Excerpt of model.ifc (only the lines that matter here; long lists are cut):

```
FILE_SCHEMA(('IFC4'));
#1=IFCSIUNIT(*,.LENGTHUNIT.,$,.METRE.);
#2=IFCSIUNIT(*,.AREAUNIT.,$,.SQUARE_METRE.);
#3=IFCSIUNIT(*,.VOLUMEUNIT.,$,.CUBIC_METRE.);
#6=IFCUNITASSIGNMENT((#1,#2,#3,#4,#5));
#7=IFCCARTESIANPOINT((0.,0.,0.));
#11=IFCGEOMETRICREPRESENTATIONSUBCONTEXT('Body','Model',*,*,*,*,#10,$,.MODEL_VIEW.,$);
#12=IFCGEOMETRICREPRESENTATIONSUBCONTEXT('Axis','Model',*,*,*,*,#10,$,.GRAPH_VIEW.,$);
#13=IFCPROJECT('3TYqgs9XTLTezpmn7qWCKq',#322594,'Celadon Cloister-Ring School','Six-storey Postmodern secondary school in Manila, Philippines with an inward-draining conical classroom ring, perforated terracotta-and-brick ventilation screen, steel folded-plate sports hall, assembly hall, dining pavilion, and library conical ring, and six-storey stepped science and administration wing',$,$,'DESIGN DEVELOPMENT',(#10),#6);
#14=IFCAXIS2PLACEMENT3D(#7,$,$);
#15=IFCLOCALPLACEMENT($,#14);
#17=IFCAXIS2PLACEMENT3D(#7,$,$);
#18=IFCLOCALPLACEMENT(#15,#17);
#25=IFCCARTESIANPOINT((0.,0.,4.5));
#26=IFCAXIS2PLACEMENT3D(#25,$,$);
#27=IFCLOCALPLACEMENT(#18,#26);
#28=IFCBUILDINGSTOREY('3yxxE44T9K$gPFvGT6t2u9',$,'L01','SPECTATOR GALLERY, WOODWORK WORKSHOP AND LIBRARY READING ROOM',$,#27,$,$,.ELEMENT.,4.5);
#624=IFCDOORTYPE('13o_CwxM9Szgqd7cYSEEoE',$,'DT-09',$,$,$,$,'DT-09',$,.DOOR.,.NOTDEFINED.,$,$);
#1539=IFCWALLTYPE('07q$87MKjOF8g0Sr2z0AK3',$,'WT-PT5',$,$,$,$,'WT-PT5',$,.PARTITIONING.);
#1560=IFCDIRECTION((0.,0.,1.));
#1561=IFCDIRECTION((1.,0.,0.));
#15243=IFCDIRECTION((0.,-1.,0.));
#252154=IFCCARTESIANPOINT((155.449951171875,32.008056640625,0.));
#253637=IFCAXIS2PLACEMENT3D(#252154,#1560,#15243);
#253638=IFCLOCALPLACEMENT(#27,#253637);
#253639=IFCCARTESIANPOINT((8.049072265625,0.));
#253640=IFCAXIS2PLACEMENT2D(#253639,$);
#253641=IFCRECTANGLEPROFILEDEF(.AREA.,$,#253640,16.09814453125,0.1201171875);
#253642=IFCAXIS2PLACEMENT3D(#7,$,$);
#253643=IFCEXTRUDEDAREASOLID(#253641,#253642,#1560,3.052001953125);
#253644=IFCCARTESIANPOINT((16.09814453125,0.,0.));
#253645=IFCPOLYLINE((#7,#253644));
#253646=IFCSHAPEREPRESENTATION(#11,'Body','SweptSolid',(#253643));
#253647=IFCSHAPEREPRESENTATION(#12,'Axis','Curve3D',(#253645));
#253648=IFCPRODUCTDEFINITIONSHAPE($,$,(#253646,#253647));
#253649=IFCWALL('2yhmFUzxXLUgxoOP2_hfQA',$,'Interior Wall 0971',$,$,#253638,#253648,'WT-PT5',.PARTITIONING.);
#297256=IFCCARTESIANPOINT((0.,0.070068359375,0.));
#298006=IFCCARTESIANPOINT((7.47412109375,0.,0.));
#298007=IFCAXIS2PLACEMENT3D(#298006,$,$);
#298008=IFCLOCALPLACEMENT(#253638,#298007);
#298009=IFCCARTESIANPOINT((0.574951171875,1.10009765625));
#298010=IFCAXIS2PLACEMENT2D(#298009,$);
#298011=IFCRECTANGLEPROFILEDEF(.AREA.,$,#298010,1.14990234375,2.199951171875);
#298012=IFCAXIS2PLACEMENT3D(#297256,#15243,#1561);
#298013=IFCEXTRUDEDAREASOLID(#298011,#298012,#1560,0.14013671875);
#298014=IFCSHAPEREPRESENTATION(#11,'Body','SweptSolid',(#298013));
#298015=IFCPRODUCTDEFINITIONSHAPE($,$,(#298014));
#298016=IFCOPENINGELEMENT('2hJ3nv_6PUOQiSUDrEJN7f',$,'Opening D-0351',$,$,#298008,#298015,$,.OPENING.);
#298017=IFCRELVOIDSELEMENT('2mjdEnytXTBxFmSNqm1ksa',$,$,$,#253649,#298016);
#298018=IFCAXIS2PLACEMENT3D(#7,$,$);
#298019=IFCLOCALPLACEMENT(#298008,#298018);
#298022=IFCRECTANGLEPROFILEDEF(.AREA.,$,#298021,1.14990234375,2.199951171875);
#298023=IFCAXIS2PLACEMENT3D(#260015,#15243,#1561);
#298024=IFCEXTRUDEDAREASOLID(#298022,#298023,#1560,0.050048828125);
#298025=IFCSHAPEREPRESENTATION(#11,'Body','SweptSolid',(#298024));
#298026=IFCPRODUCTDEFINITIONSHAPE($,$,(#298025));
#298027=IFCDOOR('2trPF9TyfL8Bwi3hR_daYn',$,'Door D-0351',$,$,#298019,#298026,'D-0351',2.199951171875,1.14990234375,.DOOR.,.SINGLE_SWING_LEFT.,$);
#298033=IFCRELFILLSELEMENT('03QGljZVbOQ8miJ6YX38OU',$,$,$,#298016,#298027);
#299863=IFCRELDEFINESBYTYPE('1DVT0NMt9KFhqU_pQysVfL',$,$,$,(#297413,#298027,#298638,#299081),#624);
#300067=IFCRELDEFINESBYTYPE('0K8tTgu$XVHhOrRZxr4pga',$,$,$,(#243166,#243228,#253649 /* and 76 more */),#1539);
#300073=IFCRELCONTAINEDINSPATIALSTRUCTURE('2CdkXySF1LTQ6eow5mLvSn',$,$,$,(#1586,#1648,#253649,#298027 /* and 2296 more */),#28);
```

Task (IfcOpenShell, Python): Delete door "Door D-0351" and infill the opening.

```python
import ifcopenshell
import ifcopenshell.api.feature
import ifcopenshell.api.root
import ifcopenshell.geom
import ifcopenshell.util.shape

model = ifcopenshell.open("model.ifc")
settings = ifcopenshell.geom.settings()


def volume(element):
    """Net volume in cubic metres, openings subtracted."""
    shape = ifcopenshell.geom.create_shape(settings, element)
    return ifcopenshell.util.shape.get_volume(shape.geometry)


door = model.by_guid("2trPF9TyfL8Bwi3hR_daYn")
opening = door.FillsVoids[0].RelatingOpeningElement
wall = opening.VoidsElements[0].RelatingBuildingElement
before = volume(wall)

ifcopenshell.api.root.remove_product(model, product=door)
ifcopenshell.api.feature.remove_feature(model, feature=opening)

after = volume(wall)

print(f"wall volume {before:.3f} -> {after:.3f} m3")

model.write("model-out.ifc")
```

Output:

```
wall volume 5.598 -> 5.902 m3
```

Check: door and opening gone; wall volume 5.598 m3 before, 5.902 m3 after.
